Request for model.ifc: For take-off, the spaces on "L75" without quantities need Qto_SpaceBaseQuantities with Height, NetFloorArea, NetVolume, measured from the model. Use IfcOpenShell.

First a look at what the model holds.

```python
import ifcopenshell
import ifcopenshell.util.element
import ifcopenshell.util.unit

model = ifcopenshell.open("model.ifc")
print(model.schema)
for unit_type in ("LENGTHUNIT", "AREAUNIT", "VOLUMEUNIT"):
    print(unit_type, ifcopenshell.util.unit.calculate_unit_scale(model, unit_type))
storey = next(s for s in model.by_type("IfcBuildingStorey") if s.Name == "L75")
spaces = [e for e in ifcopenshell.util.element.get_decomposition(storey) if e.is_a("IfcSpace")]
for e in sorted(spaces, key=lambda e: e.id()):
    print(e.id(), e.is_a(), e.Name, list(ifcopenshell.util.element.get_psets(e, qtos_only=True)), sep=" | ")
```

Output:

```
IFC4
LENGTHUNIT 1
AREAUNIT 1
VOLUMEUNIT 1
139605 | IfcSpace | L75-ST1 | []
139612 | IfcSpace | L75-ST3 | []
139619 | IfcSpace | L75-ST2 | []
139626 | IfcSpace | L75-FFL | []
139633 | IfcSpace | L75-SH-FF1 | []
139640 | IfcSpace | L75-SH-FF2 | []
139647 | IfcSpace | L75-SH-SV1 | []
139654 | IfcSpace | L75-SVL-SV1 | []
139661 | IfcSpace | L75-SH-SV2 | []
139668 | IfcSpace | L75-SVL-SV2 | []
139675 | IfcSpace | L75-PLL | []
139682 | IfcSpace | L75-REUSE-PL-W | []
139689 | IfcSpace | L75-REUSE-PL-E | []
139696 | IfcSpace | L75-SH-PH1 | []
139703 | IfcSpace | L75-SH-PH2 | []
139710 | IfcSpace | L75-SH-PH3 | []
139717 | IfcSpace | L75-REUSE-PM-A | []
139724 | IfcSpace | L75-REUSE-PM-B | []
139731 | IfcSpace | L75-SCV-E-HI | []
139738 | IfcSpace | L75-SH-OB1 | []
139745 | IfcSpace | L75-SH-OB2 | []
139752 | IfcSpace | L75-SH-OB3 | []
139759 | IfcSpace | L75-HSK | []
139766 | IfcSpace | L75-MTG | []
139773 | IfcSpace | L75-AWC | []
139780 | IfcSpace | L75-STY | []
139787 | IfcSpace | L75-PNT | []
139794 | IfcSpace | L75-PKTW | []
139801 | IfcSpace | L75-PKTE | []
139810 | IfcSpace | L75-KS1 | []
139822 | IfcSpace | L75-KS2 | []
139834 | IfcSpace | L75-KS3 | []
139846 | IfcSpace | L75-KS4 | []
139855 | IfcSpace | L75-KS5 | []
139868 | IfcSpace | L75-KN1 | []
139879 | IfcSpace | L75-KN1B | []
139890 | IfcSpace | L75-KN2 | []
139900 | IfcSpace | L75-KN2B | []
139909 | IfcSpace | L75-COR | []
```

```python
import ifcopenshell
import ifcopenshell.api.pset
import ifcopenshell.geom
import ifcopenshell.util.element
import ifcopenshell.util.shape
import ifcopenshell.util.unit

model = ifcopenshell.open("model.ifc")
unit_scale = ifcopenshell.util.unit.calculate_unit_scale(model)
area_scale = ifcopenshell.util.unit.calculate_unit_scale(model, "AREAUNIT")
volume_scale = ifcopenshell.util.unit.calculate_unit_scale(model, "VOLUMEUNIT")
settings = ifcopenshell.geom.settings()

storey = next(s for s in model.by_type("IfcBuildingStorey") if s.Name == "L75")
spaces = [e for e in ifcopenshell.util.element.get_decomposition(storey) if e.is_a("IfcSpace")]

for e in sorted(spaces, key=lambda e: e.id()):
    if ifcopenshell.util.element.get_psets(e, qtos_only=True, should_inherit=False):
        continue
    # Geometry comes back in metres, in the element's own axes.
    shape = ifcopenshell.geom.create_shape(settings, e)
    values = {
        "Height": ifcopenshell.util.shape.get_z(shape.geometry) / unit_scale,
        "NetFloorArea": ifcopenshell.util.shape.get_footprint_area(shape.geometry) / area_scale,
        "NetVolume": ifcopenshell.util.shape.get_volume(shape.geometry) / volume_scale,
    }
    qto = ifcopenshell.api.pset.add_qto(model, product=e, name="Qto_SpaceBaseQuantities")
    ifcopenshell.api.pset.edit_qto(model, qto=qto, properties=values)
    print(e.id(), {k: round(v, 3) for k, v in values.items()})

model.write("model-out.ifc")
```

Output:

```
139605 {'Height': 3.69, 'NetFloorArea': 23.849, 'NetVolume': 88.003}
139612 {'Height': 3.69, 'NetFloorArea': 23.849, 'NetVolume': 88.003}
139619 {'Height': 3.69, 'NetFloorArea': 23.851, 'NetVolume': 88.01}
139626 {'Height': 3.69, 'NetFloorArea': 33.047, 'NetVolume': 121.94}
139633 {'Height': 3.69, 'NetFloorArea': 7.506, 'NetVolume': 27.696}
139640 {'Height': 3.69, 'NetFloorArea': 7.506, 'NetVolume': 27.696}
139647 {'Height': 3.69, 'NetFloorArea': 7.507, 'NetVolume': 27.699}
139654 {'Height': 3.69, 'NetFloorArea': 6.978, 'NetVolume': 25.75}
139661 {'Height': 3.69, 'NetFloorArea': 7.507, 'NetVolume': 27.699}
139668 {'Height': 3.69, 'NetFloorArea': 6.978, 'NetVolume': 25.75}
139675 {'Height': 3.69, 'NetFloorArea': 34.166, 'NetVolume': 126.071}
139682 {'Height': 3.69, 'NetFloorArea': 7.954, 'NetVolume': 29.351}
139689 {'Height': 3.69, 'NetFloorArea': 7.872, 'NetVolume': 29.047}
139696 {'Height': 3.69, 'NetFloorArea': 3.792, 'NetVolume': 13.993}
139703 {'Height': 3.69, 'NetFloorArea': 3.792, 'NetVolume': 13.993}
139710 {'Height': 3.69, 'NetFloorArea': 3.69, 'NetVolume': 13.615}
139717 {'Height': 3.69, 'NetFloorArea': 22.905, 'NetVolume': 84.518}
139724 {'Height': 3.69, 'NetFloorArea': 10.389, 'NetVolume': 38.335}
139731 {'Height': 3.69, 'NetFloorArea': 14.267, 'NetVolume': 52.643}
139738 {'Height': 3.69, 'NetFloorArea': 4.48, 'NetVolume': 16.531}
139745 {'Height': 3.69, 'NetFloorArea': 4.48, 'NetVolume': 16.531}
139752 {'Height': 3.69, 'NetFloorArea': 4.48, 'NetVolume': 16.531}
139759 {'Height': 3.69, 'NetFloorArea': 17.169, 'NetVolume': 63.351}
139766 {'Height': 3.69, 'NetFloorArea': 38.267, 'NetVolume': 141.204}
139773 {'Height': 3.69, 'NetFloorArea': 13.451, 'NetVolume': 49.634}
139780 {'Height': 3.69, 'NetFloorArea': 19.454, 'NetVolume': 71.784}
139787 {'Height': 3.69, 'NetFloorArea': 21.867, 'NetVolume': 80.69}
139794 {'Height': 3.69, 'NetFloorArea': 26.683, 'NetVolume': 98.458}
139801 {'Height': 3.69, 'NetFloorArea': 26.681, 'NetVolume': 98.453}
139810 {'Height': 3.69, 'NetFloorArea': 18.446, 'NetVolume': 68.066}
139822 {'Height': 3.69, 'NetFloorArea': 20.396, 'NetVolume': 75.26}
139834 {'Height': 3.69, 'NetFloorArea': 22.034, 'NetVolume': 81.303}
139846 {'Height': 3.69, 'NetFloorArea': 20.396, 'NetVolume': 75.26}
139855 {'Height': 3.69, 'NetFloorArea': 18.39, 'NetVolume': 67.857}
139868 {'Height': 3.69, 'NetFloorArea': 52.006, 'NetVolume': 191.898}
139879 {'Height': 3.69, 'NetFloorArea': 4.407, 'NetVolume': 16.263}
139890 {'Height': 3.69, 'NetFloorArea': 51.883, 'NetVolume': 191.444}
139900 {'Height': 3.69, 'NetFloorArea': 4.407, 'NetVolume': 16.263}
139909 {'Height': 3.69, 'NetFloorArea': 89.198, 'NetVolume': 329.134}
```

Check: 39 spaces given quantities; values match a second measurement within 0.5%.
